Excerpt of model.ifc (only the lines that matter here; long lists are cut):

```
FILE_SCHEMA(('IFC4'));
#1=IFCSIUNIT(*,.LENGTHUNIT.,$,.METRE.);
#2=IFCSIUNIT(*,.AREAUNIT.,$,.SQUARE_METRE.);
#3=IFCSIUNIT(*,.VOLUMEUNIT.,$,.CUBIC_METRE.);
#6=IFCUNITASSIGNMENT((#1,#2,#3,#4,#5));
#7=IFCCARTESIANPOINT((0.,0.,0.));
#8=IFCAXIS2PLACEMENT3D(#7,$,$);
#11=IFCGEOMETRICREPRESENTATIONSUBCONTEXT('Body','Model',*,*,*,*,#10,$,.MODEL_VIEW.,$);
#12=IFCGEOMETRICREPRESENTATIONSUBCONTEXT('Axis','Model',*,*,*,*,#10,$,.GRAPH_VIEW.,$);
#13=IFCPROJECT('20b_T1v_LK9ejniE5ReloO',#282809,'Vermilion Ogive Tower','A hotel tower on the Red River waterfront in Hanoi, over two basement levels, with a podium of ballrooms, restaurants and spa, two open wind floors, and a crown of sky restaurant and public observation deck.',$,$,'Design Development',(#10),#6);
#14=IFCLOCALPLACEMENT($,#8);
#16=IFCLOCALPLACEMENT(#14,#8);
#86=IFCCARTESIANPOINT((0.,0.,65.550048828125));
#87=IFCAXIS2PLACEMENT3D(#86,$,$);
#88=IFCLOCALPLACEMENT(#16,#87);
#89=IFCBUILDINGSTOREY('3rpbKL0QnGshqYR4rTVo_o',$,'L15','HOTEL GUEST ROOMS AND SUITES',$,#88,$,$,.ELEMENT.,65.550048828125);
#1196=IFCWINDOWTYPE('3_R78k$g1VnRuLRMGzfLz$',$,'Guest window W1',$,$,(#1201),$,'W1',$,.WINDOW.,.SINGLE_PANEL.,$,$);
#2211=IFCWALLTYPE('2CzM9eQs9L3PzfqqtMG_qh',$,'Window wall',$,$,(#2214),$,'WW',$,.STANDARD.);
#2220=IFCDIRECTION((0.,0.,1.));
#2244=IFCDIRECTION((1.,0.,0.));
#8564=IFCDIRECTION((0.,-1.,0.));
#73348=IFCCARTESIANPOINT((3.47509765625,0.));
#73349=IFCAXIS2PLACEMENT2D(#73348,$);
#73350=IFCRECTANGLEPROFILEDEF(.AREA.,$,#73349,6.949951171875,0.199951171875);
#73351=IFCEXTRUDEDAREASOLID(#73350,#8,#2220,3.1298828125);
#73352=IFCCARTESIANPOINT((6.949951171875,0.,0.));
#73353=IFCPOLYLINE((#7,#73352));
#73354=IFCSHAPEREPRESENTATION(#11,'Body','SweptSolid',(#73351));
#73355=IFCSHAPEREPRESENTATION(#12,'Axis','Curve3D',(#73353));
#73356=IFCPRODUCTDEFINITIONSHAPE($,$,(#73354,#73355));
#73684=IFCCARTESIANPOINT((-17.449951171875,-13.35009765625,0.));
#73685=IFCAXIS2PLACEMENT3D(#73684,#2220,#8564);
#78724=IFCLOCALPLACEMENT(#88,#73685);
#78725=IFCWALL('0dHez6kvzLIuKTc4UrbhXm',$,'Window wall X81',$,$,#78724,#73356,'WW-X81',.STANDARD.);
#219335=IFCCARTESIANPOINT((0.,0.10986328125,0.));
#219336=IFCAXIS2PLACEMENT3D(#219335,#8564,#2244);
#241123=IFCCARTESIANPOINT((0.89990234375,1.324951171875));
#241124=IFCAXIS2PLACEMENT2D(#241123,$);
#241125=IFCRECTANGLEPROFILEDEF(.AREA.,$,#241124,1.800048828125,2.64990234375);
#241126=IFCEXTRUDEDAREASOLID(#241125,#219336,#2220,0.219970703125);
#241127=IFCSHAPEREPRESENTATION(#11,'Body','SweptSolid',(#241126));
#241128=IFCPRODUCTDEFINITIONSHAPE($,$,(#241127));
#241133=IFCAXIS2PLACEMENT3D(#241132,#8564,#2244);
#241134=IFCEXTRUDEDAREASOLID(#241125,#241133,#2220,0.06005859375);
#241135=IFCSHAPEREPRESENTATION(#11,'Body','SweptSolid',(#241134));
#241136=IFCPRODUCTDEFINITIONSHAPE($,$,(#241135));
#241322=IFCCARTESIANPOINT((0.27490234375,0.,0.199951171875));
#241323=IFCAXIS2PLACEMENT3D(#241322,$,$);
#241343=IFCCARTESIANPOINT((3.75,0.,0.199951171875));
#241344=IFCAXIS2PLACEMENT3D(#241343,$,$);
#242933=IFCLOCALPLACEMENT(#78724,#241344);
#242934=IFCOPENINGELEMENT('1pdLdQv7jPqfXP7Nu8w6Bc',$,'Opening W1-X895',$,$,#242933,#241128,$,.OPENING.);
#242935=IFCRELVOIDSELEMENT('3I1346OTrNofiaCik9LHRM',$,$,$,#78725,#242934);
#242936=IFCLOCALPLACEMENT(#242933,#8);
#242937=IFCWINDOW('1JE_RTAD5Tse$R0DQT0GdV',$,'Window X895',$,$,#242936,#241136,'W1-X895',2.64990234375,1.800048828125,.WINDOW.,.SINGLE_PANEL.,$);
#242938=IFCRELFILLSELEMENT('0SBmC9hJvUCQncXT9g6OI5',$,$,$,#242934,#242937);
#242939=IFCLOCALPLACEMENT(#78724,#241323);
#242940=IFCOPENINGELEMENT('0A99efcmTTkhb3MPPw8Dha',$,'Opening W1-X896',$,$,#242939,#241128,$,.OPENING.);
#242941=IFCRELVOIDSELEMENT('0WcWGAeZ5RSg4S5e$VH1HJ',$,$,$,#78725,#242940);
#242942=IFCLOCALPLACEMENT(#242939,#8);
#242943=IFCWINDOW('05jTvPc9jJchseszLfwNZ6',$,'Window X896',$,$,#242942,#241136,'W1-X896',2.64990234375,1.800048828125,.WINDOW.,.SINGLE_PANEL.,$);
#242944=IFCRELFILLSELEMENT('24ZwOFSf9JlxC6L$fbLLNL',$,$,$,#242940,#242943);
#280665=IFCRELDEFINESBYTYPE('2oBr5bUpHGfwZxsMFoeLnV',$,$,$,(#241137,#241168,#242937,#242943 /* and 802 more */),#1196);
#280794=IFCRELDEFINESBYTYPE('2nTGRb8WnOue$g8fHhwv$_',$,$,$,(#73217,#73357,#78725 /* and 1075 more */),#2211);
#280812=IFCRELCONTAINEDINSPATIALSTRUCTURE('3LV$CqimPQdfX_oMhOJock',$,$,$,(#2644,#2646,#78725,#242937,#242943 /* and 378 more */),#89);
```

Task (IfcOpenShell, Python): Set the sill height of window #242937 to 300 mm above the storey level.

```python
import numpy as np
import ifcopenshell
import ifcopenshell.api.geometry
import ifcopenshell.geom
import ifcopenshell.util.element
import ifcopenshell.util.placement
import ifcopenshell.util.shape
import ifcopenshell.util.unit

model = ifcopenshell.open("model.ifc")
unit_scale = ifcopenshell.util.unit.calculate_unit_scale(model)

window = model.by_guid("1JE_RTAD5Tse$R0DQT0GdV")
opening = window.FillsVoids[0].RelatingOpeningElement
storey = ifcopenshell.util.element.get_container(window, ifc_class="IfcBuildingStorey")
level = ifcopenshell.util.placement.get_local_placement(storey.ObjectPlacement)[2, 3]

# The opening's origin need not be at the sill, so measure its lowest point.
shape = ifcopenshell.geom.create_shape(ifcopenshell.geom.settings(), opening)
bottom = ifcopenshell.util.shape.get_shape_bottom_elevation(shape, shape.geometry) / unit_scale
dz = level + 0.3 - bottom

shift = np.array([0.0, 0.0, dz])
# The window is placed relative to its opening, so it follows when the opening moves.
matrix = ifcopenshell.util.placement.get_local_placement(opening.ObjectPlacement)
matrix[:3, 3] += shift
ifcopenshell.api.geometry.edit_object_placement(
    model, product=opening, matrix=matrix, is_si=False, should_transform_children=True
)

print(f"moved by {dz * unit_scale:+.3f} m")

model.write("model-out.ifc")
```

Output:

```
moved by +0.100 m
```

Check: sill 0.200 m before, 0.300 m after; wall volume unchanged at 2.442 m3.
